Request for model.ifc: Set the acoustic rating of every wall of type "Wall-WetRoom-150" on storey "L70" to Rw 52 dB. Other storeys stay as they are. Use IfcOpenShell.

First a look at what the model holds.

```python
import ifcopenshell
import ifcopenshell.util.element

model = ifcopenshell.open("model.ifc")
print(model.schema)
storey = next(s for s in model.by_type("IfcBuildingStorey") if s.Name == "L70")
walls = [e for e in ifcopenshell.util.element.get_decomposition(storey) if e.is_a("IfcWall")]
seen = {}
for e in walls:
    element_type = ifcopenshell.util.element.get_type(e)
    key = (element_type.Name if element_type != e and element_type else None, ifcopenshell.util.element.get_pset(e, "Pset_WallCommon", "AcousticRating"))
    seen[key] = seen.get(key, 0) + 1
for (name, value), count in sorted(seen.items(), key=str):
    print(count, "x", name, "|", value)
```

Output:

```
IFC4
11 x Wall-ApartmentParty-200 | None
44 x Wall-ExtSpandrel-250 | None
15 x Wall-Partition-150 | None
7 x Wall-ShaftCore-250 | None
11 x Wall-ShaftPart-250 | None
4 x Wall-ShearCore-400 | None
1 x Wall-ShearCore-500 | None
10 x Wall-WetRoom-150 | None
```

```python
import ifcopenshell
import ifcopenshell.api.pset
import ifcopenshell.util.element

model = ifcopenshell.open("model.ifc")

storey = next(s for s in model.by_type("IfcBuildingStorey") if s.Name == "L70")
walls = [e for e in ifcopenshell.util.element.get_decomposition(storey) if e.is_a("IfcWall")]

count = 0
for e in walls:
    element_type = ifcopenshell.util.element.get_type(e)
    if element_type in (None, e) or element_type.Name != "Wall-WetRoom-150":
        continue
    found = ifcopenshell.util.element.get_pset(e, "Pset_WallCommon", should_inherit=False)
    if found:
        pset = model.by_id(found["id"])
        if len(ifcopenshell.util.element.get_elements_by_pset(pset)) > 1:
            pset = ifcopenshell.api.pset.unshare_pset(model, products=[e], pset=pset)[0]
    else:
        pset = ifcopenshell.api.pset.add_pset(model, product=e, name="Pset_WallCommon")
    ifcopenshell.api.pset.edit_pset(model, pset=pset, properties={"AcousticRating": "Rw 52 dB"})
    count += 1

print(count, "walls updated")

model.write("model_edited.ifc")
```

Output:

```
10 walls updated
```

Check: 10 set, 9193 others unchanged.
